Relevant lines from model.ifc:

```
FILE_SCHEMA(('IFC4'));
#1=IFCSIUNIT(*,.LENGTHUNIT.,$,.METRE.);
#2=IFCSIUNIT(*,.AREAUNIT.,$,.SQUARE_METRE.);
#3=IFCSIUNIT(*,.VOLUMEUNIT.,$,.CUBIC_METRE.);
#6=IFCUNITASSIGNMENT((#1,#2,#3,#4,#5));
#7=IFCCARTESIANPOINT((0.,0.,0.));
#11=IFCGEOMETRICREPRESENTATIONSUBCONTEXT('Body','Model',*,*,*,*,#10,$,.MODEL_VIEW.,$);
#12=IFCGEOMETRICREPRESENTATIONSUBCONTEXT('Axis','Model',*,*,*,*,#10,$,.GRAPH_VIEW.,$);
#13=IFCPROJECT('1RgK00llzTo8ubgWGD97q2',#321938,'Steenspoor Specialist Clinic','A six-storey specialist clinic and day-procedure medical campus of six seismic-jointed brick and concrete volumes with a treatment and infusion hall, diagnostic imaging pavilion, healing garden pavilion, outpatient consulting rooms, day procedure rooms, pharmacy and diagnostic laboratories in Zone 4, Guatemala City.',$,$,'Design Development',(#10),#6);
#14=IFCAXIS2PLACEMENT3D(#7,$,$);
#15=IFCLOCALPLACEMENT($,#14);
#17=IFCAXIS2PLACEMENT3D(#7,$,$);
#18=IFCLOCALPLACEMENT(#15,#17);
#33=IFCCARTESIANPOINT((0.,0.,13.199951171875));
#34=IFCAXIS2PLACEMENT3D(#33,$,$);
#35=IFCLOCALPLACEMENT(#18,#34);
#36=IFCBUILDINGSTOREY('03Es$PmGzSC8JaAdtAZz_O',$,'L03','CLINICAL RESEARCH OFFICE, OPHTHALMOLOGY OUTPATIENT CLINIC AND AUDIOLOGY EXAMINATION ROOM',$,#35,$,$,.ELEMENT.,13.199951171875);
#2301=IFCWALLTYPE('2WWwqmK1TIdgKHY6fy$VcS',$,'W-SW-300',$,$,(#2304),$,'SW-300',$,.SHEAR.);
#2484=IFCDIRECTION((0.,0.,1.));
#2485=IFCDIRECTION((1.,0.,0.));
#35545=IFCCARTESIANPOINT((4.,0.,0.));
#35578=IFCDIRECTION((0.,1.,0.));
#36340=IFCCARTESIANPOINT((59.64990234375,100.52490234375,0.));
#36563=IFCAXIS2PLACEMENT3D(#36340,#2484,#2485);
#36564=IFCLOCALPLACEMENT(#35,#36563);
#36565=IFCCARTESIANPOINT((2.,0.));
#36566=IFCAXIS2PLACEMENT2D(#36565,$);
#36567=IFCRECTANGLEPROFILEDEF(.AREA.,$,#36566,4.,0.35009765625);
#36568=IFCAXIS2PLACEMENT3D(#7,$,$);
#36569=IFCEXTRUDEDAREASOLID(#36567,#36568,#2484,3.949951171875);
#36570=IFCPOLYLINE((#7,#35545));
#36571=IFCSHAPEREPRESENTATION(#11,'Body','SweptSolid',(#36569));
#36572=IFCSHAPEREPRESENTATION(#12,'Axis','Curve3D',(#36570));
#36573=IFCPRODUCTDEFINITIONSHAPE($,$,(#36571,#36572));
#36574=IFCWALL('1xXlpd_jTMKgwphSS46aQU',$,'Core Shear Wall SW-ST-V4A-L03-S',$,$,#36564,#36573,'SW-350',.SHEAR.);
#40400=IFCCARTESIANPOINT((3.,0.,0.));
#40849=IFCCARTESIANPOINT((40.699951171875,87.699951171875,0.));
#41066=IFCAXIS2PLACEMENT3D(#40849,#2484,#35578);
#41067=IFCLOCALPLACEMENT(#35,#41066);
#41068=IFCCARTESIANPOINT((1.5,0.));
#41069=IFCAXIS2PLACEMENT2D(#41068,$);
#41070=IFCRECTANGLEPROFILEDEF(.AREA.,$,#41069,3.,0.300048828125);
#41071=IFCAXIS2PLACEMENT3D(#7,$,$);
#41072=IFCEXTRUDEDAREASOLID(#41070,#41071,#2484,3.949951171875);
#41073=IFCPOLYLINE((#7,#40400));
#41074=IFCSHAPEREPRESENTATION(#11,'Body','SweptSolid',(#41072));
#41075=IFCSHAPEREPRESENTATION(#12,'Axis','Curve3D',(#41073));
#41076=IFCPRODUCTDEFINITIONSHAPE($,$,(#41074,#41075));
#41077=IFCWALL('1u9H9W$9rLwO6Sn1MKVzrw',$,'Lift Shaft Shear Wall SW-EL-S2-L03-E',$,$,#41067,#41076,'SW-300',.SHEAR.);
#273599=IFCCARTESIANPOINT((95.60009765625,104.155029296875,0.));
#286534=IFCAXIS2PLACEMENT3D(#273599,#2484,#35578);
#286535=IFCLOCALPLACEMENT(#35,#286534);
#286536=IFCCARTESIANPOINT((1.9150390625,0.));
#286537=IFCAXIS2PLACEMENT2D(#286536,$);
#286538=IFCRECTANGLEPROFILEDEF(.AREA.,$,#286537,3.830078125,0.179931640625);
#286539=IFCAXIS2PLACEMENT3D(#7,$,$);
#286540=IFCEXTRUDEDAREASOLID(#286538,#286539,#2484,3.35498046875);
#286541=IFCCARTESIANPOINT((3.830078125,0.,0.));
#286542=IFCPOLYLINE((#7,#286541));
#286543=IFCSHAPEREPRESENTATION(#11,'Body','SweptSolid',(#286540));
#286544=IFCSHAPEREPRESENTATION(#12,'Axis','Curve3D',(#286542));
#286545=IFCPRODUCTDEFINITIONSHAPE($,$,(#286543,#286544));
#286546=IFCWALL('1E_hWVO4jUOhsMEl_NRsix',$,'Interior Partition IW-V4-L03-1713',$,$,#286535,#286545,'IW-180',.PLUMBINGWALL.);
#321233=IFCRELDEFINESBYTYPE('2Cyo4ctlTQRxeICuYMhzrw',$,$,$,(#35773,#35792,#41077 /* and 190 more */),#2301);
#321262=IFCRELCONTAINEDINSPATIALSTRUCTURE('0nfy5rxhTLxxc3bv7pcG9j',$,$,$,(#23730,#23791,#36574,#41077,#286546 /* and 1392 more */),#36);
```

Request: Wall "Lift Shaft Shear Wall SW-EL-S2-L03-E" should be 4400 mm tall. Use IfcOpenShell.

```python
import ifcopenshell
import ifcopenshell.geom
import ifcopenshell.util.representation
import ifcopenshell.util.shape
import ifcopenshell.util.unit

model = ifcopenshell.open("model.ifc")
unit_scale = ifcopenshell.util.unit.calculate_unit_scale(model)
settings = ifcopenshell.geom.settings()


def volume(element):
    """Net volume in cubic metres, openings subtracted."""
    shape = ifcopenshell.geom.create_shape(settings, element)
    return ifcopenshell.util.shape.get_volume(shape.geometry)


wall = model.by_id(41077)
before = volume(wall)

body = ifcopenshell.util.representation.get_representation(wall, "Model", "Body")
solid = body.Items[0]
old_height = solid.Depth
solid.Depth = 4.4 / unit_scale
after = volume(wall)

print(f"height {old_height:g} -> {solid.Depth:g}, volume {before:.3f} -> {after:.3f} m3")

model.write("model_rev.ifc")
```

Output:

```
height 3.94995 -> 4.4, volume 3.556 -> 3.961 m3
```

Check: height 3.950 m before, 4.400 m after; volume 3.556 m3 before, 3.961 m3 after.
